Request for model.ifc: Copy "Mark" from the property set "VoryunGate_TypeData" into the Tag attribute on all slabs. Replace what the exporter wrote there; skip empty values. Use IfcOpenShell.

First a look at what the model holds.

```python
import ifcopenshell
import ifcopenshell.util.element

model = ifcopenshell.open("model.ifc")
print(model.schema)
slabs = model.by_type("IfcSlab")
print(len(slabs), "slabs")
for e in slabs[:8]:
    source = ifcopenshell.util.element.get_pset(e, "VoryunGate_TypeData", "Mark")
    target = e.Tag
    print(e.id(), repr(source), repr(target), sep=" | ")
```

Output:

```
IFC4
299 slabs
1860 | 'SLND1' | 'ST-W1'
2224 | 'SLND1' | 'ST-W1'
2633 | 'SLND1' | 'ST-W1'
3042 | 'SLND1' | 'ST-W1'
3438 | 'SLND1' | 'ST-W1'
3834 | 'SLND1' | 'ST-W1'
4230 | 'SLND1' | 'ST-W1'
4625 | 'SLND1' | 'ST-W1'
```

```python
import ifcopenshell
import ifcopenshell.util.element

model = ifcopenshell.open("model.ifc")

count = 0
for e in model.by_type("IfcSlab"):
    value = ifcopenshell.util.element.get_pset(e, "VoryunGate_TypeData", "Mark")
    current = e.Tag
    if not value or not value.strip() or current == value:
        continue
    e.Tag = value
    count += 1

print(count, "slabs updated")

model.write("model-out.ifc")
```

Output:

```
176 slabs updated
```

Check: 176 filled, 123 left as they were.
